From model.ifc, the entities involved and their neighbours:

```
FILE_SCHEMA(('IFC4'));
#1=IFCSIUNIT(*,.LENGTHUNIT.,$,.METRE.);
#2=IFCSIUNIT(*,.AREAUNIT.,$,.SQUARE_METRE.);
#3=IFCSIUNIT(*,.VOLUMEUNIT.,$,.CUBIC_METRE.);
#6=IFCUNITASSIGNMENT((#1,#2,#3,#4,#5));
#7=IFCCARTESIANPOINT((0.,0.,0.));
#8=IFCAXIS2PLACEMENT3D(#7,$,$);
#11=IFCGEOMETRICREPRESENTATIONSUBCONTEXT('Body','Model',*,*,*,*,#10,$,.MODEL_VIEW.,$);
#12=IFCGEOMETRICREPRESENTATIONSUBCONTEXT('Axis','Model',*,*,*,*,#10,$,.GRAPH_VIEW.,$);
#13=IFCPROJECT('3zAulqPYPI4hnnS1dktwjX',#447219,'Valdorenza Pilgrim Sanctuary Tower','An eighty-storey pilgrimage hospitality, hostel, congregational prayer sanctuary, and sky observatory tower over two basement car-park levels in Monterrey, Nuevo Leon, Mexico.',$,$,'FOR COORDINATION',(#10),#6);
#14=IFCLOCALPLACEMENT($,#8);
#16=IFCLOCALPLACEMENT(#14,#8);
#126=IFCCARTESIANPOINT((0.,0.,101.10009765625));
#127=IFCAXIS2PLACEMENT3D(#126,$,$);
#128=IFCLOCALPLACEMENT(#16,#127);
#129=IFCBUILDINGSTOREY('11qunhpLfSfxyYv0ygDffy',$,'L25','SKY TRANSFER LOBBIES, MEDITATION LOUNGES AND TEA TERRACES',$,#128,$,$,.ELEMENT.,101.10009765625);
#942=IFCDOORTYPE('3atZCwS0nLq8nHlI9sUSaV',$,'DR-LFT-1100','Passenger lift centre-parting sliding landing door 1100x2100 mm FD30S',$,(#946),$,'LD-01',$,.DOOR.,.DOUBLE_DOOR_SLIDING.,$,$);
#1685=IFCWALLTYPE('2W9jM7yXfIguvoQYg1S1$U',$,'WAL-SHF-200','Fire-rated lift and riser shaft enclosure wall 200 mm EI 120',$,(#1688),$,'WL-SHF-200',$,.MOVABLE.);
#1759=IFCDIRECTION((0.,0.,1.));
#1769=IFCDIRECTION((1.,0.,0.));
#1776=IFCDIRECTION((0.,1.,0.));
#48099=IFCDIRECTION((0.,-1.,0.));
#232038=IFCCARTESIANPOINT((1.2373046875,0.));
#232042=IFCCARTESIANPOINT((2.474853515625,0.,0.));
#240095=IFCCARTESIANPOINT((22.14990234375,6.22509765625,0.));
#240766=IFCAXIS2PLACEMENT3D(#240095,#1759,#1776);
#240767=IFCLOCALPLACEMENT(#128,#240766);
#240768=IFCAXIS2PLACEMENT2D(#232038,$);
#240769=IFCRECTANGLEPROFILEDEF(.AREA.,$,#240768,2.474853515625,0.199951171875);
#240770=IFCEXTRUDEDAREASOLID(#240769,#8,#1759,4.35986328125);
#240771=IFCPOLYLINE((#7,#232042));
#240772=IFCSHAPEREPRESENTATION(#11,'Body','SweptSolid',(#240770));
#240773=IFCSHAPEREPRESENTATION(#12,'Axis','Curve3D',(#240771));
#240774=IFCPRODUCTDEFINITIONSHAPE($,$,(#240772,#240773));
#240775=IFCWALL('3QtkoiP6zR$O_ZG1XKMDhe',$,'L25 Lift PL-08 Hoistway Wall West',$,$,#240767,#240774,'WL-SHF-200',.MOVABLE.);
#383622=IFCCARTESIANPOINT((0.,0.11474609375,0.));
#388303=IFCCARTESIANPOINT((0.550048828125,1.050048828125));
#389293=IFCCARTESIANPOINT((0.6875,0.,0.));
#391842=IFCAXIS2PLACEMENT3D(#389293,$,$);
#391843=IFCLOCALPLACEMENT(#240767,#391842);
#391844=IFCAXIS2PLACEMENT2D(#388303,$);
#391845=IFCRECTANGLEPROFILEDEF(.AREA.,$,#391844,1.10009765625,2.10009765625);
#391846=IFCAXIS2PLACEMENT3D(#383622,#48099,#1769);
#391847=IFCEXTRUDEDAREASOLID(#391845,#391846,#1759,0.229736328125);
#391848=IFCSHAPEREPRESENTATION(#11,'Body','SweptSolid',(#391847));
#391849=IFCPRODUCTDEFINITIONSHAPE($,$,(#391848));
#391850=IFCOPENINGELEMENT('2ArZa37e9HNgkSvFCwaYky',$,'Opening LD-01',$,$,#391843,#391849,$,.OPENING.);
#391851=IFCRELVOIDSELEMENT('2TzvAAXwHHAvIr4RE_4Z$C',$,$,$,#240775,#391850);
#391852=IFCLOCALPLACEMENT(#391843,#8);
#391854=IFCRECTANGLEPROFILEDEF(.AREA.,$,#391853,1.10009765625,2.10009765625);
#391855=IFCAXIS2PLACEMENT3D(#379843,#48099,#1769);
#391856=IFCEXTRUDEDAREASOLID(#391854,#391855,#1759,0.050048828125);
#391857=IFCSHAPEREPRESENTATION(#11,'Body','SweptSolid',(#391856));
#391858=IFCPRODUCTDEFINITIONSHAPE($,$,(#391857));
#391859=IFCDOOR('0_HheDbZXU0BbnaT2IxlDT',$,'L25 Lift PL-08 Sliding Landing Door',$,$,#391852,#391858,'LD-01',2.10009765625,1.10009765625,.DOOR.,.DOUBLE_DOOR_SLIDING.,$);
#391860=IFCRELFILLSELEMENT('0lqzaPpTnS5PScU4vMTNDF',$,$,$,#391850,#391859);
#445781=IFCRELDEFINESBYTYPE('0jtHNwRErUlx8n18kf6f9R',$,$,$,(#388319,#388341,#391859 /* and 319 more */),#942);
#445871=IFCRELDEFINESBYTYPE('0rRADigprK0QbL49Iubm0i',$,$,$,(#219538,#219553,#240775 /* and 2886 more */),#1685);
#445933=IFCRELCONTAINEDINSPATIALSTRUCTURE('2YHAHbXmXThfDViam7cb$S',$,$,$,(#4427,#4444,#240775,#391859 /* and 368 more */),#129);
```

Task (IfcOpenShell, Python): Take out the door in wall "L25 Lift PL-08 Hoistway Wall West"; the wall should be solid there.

```python
import ifcopenshell
import ifcopenshell.api.feature
import ifcopenshell.api.root
import ifcopenshell.geom
import ifcopenshell.util.shape

model = ifcopenshell.open("model.ifc")
settings = ifcopenshell.geom.settings()


def volume(element):
    """Net volume in cubic metres, openings subtracted."""
    shape = ifcopenshell.geom.create_shape(settings, element)
    return ifcopenshell.util.shape.get_volume(shape.geometry)


door = model.by_guid("0_HheDbZXU0BbnaT2IxlDT")
opening = door.FillsVoids[0].RelatingOpeningElement
wall = opening.VoidsElements[0].RelatingBuildingElement
before = volume(wall)

ifcopenshell.api.root.remove_product(model, product=door)
ifcopenshell.api.feature.remove_feature(model, feature=opening)

after = volume(wall)

print(f"wall volume {before:.3f} -> {after:.3f} m3")

model.write("model_rev.ifc")
```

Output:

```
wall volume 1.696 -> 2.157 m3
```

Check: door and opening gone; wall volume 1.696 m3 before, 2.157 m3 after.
